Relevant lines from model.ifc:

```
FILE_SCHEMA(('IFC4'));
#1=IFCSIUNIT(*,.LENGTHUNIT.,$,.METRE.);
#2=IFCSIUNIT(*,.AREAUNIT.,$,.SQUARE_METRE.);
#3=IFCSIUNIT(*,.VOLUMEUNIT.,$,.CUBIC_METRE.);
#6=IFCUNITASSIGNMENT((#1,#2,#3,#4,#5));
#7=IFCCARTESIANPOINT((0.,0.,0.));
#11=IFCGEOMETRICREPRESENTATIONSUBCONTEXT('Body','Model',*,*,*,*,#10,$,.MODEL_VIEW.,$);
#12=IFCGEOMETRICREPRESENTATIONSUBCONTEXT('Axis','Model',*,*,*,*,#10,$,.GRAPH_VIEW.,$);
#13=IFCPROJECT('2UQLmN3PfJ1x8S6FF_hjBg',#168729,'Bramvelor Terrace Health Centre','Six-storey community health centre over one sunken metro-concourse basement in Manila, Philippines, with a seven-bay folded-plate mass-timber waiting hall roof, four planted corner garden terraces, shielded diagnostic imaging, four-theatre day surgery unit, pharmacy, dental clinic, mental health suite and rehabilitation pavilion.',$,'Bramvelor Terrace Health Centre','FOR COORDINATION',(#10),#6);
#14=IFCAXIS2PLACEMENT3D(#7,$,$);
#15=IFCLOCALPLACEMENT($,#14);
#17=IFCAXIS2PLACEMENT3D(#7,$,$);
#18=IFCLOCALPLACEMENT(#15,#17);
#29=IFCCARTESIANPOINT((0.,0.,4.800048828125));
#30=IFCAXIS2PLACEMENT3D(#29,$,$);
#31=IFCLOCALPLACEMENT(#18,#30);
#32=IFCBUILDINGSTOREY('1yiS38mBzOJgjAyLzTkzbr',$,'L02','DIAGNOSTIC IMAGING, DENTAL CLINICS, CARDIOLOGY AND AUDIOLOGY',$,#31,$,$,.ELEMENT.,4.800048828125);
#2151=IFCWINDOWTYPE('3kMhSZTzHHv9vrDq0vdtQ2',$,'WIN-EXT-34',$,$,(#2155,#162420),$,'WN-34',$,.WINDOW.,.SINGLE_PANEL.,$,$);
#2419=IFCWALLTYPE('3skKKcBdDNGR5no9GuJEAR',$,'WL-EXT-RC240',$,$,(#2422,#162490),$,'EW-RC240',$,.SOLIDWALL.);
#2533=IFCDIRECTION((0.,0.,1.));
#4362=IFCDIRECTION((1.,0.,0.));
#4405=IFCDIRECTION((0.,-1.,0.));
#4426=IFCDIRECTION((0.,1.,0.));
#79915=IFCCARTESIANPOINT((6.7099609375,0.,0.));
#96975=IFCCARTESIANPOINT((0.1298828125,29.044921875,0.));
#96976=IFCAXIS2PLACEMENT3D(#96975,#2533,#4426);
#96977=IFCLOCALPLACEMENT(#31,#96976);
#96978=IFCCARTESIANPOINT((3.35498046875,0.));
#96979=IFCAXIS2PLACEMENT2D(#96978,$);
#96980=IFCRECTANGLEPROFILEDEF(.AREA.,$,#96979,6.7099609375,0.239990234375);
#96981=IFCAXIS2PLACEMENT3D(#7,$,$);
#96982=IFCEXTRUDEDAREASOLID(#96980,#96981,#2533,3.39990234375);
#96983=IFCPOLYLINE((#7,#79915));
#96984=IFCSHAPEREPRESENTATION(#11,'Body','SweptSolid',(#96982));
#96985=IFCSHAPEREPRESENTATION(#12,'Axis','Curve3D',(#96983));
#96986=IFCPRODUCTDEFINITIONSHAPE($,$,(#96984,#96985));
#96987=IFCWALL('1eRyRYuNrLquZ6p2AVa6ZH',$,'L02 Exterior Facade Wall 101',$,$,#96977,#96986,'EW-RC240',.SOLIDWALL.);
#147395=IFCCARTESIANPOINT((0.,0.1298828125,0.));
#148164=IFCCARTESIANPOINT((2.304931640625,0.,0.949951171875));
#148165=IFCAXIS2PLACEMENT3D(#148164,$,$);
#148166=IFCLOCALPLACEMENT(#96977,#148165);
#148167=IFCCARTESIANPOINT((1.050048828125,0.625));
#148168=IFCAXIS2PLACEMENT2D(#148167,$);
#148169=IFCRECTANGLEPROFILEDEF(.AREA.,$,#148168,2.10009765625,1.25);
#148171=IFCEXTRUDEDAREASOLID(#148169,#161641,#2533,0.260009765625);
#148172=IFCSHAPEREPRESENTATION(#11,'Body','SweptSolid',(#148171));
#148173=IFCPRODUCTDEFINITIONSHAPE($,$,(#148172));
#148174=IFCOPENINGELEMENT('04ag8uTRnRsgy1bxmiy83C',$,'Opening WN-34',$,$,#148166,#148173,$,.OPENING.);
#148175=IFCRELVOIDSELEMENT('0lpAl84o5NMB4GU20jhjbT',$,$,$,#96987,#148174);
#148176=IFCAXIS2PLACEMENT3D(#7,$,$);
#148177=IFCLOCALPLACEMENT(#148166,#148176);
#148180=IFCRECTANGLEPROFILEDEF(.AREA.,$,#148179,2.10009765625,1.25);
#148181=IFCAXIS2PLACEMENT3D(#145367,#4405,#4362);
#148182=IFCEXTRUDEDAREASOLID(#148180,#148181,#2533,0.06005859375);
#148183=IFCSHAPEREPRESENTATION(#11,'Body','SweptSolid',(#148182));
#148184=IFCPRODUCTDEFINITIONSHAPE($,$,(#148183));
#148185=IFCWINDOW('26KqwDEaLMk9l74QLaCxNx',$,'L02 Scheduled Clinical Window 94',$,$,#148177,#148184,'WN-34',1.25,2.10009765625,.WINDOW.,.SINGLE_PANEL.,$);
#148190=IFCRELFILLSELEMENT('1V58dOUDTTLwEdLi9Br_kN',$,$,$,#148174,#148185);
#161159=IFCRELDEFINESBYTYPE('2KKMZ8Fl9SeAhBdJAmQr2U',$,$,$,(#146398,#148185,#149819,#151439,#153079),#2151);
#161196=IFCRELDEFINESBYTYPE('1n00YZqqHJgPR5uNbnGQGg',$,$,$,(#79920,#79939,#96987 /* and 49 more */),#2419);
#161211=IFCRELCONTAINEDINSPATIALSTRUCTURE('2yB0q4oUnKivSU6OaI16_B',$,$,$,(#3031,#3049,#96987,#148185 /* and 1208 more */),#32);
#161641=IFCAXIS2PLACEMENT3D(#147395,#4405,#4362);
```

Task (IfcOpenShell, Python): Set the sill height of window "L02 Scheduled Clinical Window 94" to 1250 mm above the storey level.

```python
import numpy as np
import ifcopenshell
import ifcopenshell.api.geometry
import ifcopenshell.geom
import ifcopenshell.util.element
import ifcopenshell.util.placement
import ifcopenshell.util.shape
import ifcopenshell.util.unit

model = ifcopenshell.open("model.ifc")
unit_scale = ifcopenshell.util.unit.calculate_unit_scale(model)

window = model.by_guid("26KqwDEaLMk9l74QLaCxNx")
opening = window.FillsVoids[0].RelatingOpeningElement
storey = ifcopenshell.util.element.get_container(window, ifc_class="IfcBuildingStorey")
level = ifcopenshell.util.placement.get_local_placement(storey.ObjectPlacement)[2, 3]

# The opening's origin need not be at the sill, so measure its lowest point.
shape = ifcopenshell.geom.create_shape(ifcopenshell.geom.settings(), opening)
bottom = ifcopenshell.util.shape.get_shape_bottom_elevation(shape, shape.geometry) / unit_scale
dz = level + 1.25 / unit_scale - bottom

shift = np.array([0.0, 0.0, dz])
# The window is placed relative to its opening, so it follows when the opening moves.
matrix = ifcopenshell.util.placement.get_local_placement(opening.ObjectPlacement)
matrix[:3, 3] += shift
ifcopenshell.api.geometry.edit_object_placement(
    model, product=opening, matrix=matrix, is_si=False, should_transform_children=True
)

print(f"moved by {dz * unit_scale:+.3f} m")

model.write("model_rev.ifc")
```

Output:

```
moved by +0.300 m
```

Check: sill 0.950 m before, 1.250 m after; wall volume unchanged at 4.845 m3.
